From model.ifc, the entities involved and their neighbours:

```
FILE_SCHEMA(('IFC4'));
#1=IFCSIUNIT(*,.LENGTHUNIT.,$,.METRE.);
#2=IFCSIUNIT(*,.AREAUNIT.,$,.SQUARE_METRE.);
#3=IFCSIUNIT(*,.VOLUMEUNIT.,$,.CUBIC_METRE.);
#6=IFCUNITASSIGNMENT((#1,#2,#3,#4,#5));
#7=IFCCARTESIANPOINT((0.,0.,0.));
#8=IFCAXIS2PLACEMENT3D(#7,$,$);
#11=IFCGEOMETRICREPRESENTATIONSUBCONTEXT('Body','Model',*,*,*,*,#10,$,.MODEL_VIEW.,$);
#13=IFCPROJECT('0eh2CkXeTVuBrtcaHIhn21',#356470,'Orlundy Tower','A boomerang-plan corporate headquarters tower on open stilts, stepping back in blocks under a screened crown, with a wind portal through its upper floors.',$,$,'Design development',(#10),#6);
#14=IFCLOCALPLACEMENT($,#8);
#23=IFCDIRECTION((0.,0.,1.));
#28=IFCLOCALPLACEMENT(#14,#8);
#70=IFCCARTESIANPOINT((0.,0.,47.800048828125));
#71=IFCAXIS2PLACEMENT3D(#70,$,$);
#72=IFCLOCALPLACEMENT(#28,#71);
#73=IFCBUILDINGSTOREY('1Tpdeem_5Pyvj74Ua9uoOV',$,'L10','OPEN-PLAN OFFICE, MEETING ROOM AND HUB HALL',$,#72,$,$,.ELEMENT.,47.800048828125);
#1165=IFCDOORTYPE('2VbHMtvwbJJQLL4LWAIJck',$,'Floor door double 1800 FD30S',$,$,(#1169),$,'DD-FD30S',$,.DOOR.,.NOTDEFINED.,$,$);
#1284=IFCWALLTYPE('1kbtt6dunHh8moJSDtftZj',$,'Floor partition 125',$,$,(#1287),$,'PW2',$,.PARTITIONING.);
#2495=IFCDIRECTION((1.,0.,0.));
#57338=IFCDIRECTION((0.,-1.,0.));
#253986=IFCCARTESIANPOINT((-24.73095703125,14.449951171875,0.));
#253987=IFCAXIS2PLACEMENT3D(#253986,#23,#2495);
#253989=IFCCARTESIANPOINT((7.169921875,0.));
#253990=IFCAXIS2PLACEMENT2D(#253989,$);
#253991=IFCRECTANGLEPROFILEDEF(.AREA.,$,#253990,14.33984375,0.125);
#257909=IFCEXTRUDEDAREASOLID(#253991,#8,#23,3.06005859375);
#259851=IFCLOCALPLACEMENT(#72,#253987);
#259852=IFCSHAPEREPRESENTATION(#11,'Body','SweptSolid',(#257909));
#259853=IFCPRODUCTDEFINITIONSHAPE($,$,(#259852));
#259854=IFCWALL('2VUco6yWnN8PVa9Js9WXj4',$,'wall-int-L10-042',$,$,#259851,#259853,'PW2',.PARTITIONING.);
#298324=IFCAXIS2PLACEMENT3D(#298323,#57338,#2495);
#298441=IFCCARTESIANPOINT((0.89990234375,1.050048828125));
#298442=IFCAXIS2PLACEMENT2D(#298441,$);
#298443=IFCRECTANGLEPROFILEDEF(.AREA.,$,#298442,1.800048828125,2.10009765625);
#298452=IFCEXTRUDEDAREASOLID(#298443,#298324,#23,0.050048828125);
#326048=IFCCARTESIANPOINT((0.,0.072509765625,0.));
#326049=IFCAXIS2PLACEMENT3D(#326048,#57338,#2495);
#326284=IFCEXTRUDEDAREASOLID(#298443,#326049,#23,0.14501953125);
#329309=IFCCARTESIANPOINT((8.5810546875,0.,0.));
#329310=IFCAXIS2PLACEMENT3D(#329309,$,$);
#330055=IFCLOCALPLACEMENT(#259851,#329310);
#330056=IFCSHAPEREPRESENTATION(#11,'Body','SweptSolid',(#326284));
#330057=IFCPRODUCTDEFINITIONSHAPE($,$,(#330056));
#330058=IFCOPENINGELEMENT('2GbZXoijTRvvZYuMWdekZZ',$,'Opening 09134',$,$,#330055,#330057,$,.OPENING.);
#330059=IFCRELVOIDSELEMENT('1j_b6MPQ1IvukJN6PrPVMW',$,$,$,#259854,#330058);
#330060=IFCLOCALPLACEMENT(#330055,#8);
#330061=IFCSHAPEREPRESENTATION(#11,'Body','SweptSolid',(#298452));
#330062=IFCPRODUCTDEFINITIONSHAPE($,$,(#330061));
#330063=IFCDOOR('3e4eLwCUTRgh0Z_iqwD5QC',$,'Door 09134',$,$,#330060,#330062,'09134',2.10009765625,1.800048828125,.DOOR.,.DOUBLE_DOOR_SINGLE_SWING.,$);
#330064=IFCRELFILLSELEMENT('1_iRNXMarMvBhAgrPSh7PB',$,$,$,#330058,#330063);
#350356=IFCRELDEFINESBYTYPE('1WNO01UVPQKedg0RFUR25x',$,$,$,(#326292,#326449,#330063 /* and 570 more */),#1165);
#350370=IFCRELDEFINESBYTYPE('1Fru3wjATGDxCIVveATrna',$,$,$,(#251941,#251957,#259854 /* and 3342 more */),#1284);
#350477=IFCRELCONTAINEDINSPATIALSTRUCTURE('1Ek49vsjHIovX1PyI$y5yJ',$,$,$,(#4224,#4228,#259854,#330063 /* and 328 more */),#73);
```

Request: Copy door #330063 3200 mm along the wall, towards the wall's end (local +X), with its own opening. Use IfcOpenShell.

```python
import ifcopenshell
import ifcopenshell.api.feature
import ifcopenshell.api.geometry
import ifcopenshell.api.root
import ifcopenshell.geom
import ifcopenshell.util.element
import ifcopenshell.util.placement
import ifcopenshell.util.shape

model = ifcopenshell.open("model.ifc")
settings = ifcopenshell.geom.settings()


def volume(element):
    """Net volume in cubic metres, openings subtracted."""
    shape = ifcopenshell.geom.create_shape(settings, element)
    return ifcopenshell.util.shape.get_volume(shape.geometry)


door = model.by_id(330063)
opening = door.FillsVoids[0].RelatingOpeningElement
wall = opening.VoidsElements[0].RelatingBuildingElement
before = volume(wall)
shift = ifcopenshell.util.placement.get_local_placement(wall.ObjectPlacement)[:3, 0] * 3.2

# copy_class copies the void relationship, type, container and properties, but no geometry.
new_opening = ifcopenshell.api.root.copy_class(model, product=opening)
new_opening.Representation = ifcopenshell.util.element.copy_deep(
    model, opening.Representation, exclude=["IfcGeometricRepresentationContext", "IfcRepresentationMap"]
)
new_door = ifcopenshell.api.root.copy_class(model, product=door)
new_door.Representation = ifcopenshell.util.element.copy_deep(
    model, door.Representation, exclude=["IfcGeometricRepresentationContext", "IfcRepresentationMap"]
)
new_door.Tag = None
ifcopenshell.api.feature.add_filling(model, opening=new_opening, element=new_door)

for old, new in ((opening, new_opening), (door, new_door)):
    matrix = ifcopenshell.util.placement.get_local_placement(old.ObjectPlacement)
    matrix[:3, 3] += shift
    ifcopenshell.api.geometry.edit_object_placement(model, product=new, matrix=matrix, is_si=False)

after = volume(wall)

print(f"wall volume {before:.3f} -> {after:.3f} m3")

model.write("model_v2.ifc")
```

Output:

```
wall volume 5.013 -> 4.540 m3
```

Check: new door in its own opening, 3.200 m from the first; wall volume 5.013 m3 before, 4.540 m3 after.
